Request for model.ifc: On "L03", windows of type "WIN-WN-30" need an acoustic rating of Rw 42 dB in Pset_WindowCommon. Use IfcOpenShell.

First a look at what the model holds.

```python
import ifcopenshell
import ifcopenshell.util.element

model = ifcopenshell.open("model.ifc")
print(model.schema)
storey = next(s for s in model.by_type("IfcBuildingStorey") if s.Name == "L03")
windows = [e for e in ifcopenshell.util.element.get_decomposition(storey) if e.is_a("IfcWindow")]
seen = {}
for e in windows:
    element_type = ifcopenshell.util.element.get_type(e)
    key = (element_type.Name if element_type != e and element_type else None, ifcopenshell.util.element.get_pset(e, "Pset_WindowCommon", "AcousticRating"))
    seen[key] = seen.get(key, 0) + 1
for (name, value), count in sorted(seen.items(), key=str):
    print(count, "x", name, "|", value)
```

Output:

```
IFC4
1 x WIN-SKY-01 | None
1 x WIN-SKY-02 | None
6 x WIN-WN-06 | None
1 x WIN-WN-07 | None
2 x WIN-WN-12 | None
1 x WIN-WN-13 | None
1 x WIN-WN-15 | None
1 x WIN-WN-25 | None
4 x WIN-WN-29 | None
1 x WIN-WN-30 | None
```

```python
import ifcopenshell
import ifcopenshell.api.pset
import ifcopenshell.util.element

model = ifcopenshell.open("model.ifc")

storey = next(s for s in model.by_type("IfcBuildingStorey") if s.Name == "L03")
windows = [e for e in ifcopenshell.util.element.get_decomposition(storey) if e.is_a("IfcWindow")]

count = 0
for e in windows:
    element_type = ifcopenshell.util.element.get_type(e)
    if element_type in (None, e) or element_type.Name != "WIN-WN-30":
        continue
    # add_pset returns the element's existing set when there is one.
    pset = ifcopenshell.api.pset.add_pset(model, product=e, name="Pset_WindowCommon")
    ifcopenshell.api.pset.edit_pset(model, pset=pset, properties={"AcousticRating": "Rw 42 dB"})
    count += 1

print(count, "windows updated")

model.write("model-out.ifc")
```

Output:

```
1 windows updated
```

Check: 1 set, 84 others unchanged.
